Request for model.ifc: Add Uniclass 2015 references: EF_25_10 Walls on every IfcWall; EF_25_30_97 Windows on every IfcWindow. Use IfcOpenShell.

First a look at what the model holds.

```python
import ifcopenshell

model = ifcopenshell.open("model.ifc")
print(model.schema)
print("classifications:", [c.Name for c in model.by_type("IfcClassification")])
for ifc_class in ("IfcDoor", "IfcRoof", "IfcStair", "IfcWall", "IfcWindow"):
    print(ifc_class, len(model.by_type(ifc_class)))
```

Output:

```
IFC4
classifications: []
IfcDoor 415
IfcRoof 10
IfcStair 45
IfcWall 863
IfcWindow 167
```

```python
import ifcopenshell
import ifcopenshell.api.classification

model = ifcopenshell.open("model.ifc")

system = ifcopenshell.api.classification.add_classification(model, classification="Uniclass 2015")

codes = {
    "IfcWall": ("EF_25_10", "Walls"),
    "IfcWindow": ("EF_25_30_97", "Windows"),
}
for ifc_class, (code, name) in codes.items():
    products = model.by_type(ifc_class)
    ifcopenshell.api.classification.add_reference(
        model, products=products, classification=system, identification=code, name=name
    )
    print(code, len(products))

model.write("model_rev.ifc")
```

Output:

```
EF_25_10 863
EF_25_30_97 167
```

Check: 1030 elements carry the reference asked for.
